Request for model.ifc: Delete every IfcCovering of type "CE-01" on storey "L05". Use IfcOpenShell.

First a look at what the model holds.

```python
import ifcopenshell
import ifcopenshell.util.element

model = ifcopenshell.open("model.ifc")
print(model.schema)
storey = next(s for s in model.by_type("IfcBuildingStorey") if s.Name == "L05")
coverings = [e for e in ifcopenshell.util.element.get_decomposition(storey) if e.is_a("IfcCovering")]
seen = {}
for e in coverings:
    element_type = ifcopenshell.util.element.get_type(e)
    name = element_type.Name if element_type not in (None, e) else None
    seen[name] = seen.get(name, 0) + 1
for name, count in sorted(seen.items(), key=str):
    print(count, "x", name)
```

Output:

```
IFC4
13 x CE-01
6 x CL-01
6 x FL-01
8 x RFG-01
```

```python
import ifcopenshell
import ifcopenshell.api.root
import ifcopenshell.util.element

model = ifcopenshell.open("model.ifc")

storey = next(s for s in model.by_type("IfcBuildingStorey") if s.Name == "L05")
coverings = [e for e in ifcopenshell.util.element.get_decomposition(storey) if e.is_a("IfcCovering")]
targets = [e for e in coverings if (t := ifcopenshell.util.element.get_type(e)) not in (None, e) and t.Name == "CE-01"]

for e in targets:
    ifcopenshell.api.root.remove_product(model, product=e)
print(len(targets), "removed")

model.write("model-out.ifc")
```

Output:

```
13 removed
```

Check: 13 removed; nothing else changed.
